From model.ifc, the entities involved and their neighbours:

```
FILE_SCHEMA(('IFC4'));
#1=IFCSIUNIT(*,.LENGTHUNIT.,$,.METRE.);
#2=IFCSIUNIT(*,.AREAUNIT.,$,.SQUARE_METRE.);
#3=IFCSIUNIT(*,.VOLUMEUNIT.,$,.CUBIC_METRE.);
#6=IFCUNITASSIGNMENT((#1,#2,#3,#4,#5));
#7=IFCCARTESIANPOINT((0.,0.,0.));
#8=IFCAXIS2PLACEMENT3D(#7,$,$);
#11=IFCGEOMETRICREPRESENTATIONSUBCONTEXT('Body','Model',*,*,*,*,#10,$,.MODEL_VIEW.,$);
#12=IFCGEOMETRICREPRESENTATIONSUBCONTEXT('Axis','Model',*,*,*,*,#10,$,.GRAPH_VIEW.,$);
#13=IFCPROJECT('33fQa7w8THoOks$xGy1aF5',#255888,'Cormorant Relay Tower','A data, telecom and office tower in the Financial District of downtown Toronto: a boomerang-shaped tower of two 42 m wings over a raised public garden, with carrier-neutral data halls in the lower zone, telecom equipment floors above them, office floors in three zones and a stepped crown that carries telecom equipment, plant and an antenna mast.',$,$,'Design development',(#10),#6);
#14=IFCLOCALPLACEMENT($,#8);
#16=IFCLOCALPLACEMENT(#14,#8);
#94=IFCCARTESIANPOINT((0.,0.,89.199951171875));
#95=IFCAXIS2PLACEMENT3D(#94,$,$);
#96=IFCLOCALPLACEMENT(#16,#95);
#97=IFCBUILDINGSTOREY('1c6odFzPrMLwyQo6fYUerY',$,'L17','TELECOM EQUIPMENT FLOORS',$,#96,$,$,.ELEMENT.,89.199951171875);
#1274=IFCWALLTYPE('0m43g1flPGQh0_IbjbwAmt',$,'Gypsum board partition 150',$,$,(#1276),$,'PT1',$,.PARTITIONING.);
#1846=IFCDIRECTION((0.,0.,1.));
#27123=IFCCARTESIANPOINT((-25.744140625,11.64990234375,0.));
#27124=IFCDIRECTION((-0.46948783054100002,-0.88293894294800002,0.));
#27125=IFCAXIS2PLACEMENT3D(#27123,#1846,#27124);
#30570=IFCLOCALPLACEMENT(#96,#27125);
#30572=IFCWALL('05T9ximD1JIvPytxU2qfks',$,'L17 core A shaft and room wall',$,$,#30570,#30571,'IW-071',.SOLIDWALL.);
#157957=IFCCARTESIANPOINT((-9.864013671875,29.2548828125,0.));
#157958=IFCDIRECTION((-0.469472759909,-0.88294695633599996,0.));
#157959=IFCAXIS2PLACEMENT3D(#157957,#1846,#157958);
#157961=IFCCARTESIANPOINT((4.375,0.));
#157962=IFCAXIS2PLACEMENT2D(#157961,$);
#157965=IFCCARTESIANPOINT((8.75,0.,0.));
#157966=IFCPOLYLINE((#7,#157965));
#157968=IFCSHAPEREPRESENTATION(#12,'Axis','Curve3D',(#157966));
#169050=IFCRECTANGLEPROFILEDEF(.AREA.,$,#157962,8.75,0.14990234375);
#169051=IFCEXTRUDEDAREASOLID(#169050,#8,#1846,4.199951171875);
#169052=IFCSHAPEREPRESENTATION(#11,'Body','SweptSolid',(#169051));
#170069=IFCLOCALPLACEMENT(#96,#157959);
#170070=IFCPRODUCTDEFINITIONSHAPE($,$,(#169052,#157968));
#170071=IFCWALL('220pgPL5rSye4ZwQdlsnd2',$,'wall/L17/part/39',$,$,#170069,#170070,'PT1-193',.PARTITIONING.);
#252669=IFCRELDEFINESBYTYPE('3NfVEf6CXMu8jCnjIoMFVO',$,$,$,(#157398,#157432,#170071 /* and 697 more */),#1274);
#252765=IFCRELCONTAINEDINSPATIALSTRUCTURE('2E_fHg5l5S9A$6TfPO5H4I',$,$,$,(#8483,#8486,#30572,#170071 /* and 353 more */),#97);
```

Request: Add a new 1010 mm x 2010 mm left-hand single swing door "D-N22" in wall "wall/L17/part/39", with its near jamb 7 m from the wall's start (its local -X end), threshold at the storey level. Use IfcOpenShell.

```python
import numpy as np
import ifcopenshell
import ifcopenshell.api.feature
import ifcopenshell.api.geometry
import ifcopenshell.api.root
import ifcopenshell.api.spatial
import ifcopenshell.geom
import ifcopenshell.util.element
import ifcopenshell.util.placement
import ifcopenshell.util.representation
import ifcopenshell.util.shape
import ifcopenshell.util.unit

model = ifcopenshell.open("model.ifc")
unit_scale = ifcopenshell.util.unit.calculate_unit_scale(model)
settings = ifcopenshell.geom.settings()


def volume(element):
    """Net volume in cubic metres, openings subtracted."""
    shape = ifcopenshell.geom.create_shape(settings, element)
    return ifcopenshell.util.shape.get_volume(shape.geometry)


wall = model.by_guid("220pgPL5rSye4ZwQdlsnd2")
storey = ifcopenshell.util.element.get_container(wall, ifc_class="IfcBuildingStorey")
context = ifcopenshell.util.representation.get_context(model, "Model", "Body", "MODEL_VIEW")
before = volume(wall)

width, height, from_end, sill = 1.01, 2.01, 7, 0.0  # metres

# The wall runs along its own X axis, and the end named is its -X end.
wall_shape = ifcopenshell.geom.create_shape(settings, wall)
x, y, z = ifcopenshell.util.shape.get_vertices(wall_shape.geometry).T
start = x.min() + from_end
face, thickness = float(y.min()), float(y.max() - y.min())
wall_matrix = ifcopenshell.util.placement.get_local_placement(wall.ObjectPlacement)
level = ifcopenshell.util.placement.get_local_placement(storey.ObjectPlacement)[2, 3]


def in_wall(x, y):
    """Placement at x, y metres in the wall's axes, at sill height."""
    matrix = wall_matrix.copy()
    matrix[:, 3] = wall_matrix @ np.array([x / unit_scale, y / unit_scale, 0.0, 1.0])
    matrix[2, 3] = level + sill / unit_scale
    return matrix


# Opening: a box that overshoots both wall faces by 50 mm.
opening = ifcopenshell.api.root.create_entity(model, ifc_class="IfcOpeningElement", predefined_type="OPENING")
box = ifcopenshell.api.geometry.add_wall_representation(
    model, context=context, length=width, height=height, thickness=thickness + 0.1
)
ifcopenshell.api.geometry.assign_representation(model, product=opening, representation=box)
ifcopenshell.api.geometry.edit_object_placement(model, product=opening, matrix=in_wall(start, face - 0.05), is_si=False)
ifcopenshell.api.feature.add_feature(model, feature=opening, element=wall)

door = ifcopenshell.api.root.create_entity(model, ifc_class="IfcDoor", name="D-N22", predefined_type="DOOR")
door.OverallWidth, door.OverallHeight = width / unit_scale, height / unit_scale
door.OperationType = "SINGLE_SWING_LEFT"
body = ifcopenshell.api.geometry.add_door_representation(
    model,
    context=context,
    overall_width=door.OverallWidth,
    overall_height=door.OverallHeight,
    operation_type="SINGLE_SWING_LEFT",
    lining_properties={"LiningDepth": thickness / unit_scale, "ThresholdDepth": thickness / unit_scale},
)
ifcopenshell.api.geometry.assign_representation(model, product=door, representation=body)
ifcopenshell.api.spatial.assign_container(model, products=[door], relating_structure=storey)
ifcopenshell.api.feature.add_filling(model, opening=opening, element=door)

# The lining spans the wall, so the door starts at the wall face.
ifcopenshell.api.geometry.edit_object_placement(model, product=door, matrix=in_wall(start, face), is_si=False)

after = volume(wall)

print(f"wall volume {before:.3f} -> {after:.3f} m3")

model.write("model_edited.ifc")
```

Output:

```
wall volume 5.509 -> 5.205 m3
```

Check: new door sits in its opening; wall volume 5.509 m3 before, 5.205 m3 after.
